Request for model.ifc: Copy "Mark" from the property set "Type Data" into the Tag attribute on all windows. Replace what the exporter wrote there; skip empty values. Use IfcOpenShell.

First a look at what the model holds.

```python
import ifcopenshell
import ifcopenshell.util.element

model = ifcopenshell.open("model.ifc")
print(model.schema)
windows = model.by_type("IfcWindow")
print(len(windows), "windows")
for e in windows[:8]:
    source = ifcopenshell.util.element.get_pset(e, "Type Data", "Mark")
    target = e.Tag
    print(e.id(), repr(source), repr(target), sep=" | ")
```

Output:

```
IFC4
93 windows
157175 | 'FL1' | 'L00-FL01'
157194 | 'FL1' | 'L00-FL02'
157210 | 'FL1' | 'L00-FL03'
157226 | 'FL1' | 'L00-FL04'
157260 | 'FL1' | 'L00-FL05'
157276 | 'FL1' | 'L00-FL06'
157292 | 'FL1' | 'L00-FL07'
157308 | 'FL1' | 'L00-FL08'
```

```python
import ifcopenshell
import ifcopenshell.util.element

model = ifcopenshell.open("model.ifc")

count = 0
for e in model.by_type("IfcWindow"):
    value = ifcopenshell.util.element.get_pset(e, "Type Data", "Mark")
    current = e.Tag
    if not value or not value.strip() or current == value:
        continue
    e.Tag = value
    count += 1

print(count, "windows updated")

model.write("model_v2.ifc")
```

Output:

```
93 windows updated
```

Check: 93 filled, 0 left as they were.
